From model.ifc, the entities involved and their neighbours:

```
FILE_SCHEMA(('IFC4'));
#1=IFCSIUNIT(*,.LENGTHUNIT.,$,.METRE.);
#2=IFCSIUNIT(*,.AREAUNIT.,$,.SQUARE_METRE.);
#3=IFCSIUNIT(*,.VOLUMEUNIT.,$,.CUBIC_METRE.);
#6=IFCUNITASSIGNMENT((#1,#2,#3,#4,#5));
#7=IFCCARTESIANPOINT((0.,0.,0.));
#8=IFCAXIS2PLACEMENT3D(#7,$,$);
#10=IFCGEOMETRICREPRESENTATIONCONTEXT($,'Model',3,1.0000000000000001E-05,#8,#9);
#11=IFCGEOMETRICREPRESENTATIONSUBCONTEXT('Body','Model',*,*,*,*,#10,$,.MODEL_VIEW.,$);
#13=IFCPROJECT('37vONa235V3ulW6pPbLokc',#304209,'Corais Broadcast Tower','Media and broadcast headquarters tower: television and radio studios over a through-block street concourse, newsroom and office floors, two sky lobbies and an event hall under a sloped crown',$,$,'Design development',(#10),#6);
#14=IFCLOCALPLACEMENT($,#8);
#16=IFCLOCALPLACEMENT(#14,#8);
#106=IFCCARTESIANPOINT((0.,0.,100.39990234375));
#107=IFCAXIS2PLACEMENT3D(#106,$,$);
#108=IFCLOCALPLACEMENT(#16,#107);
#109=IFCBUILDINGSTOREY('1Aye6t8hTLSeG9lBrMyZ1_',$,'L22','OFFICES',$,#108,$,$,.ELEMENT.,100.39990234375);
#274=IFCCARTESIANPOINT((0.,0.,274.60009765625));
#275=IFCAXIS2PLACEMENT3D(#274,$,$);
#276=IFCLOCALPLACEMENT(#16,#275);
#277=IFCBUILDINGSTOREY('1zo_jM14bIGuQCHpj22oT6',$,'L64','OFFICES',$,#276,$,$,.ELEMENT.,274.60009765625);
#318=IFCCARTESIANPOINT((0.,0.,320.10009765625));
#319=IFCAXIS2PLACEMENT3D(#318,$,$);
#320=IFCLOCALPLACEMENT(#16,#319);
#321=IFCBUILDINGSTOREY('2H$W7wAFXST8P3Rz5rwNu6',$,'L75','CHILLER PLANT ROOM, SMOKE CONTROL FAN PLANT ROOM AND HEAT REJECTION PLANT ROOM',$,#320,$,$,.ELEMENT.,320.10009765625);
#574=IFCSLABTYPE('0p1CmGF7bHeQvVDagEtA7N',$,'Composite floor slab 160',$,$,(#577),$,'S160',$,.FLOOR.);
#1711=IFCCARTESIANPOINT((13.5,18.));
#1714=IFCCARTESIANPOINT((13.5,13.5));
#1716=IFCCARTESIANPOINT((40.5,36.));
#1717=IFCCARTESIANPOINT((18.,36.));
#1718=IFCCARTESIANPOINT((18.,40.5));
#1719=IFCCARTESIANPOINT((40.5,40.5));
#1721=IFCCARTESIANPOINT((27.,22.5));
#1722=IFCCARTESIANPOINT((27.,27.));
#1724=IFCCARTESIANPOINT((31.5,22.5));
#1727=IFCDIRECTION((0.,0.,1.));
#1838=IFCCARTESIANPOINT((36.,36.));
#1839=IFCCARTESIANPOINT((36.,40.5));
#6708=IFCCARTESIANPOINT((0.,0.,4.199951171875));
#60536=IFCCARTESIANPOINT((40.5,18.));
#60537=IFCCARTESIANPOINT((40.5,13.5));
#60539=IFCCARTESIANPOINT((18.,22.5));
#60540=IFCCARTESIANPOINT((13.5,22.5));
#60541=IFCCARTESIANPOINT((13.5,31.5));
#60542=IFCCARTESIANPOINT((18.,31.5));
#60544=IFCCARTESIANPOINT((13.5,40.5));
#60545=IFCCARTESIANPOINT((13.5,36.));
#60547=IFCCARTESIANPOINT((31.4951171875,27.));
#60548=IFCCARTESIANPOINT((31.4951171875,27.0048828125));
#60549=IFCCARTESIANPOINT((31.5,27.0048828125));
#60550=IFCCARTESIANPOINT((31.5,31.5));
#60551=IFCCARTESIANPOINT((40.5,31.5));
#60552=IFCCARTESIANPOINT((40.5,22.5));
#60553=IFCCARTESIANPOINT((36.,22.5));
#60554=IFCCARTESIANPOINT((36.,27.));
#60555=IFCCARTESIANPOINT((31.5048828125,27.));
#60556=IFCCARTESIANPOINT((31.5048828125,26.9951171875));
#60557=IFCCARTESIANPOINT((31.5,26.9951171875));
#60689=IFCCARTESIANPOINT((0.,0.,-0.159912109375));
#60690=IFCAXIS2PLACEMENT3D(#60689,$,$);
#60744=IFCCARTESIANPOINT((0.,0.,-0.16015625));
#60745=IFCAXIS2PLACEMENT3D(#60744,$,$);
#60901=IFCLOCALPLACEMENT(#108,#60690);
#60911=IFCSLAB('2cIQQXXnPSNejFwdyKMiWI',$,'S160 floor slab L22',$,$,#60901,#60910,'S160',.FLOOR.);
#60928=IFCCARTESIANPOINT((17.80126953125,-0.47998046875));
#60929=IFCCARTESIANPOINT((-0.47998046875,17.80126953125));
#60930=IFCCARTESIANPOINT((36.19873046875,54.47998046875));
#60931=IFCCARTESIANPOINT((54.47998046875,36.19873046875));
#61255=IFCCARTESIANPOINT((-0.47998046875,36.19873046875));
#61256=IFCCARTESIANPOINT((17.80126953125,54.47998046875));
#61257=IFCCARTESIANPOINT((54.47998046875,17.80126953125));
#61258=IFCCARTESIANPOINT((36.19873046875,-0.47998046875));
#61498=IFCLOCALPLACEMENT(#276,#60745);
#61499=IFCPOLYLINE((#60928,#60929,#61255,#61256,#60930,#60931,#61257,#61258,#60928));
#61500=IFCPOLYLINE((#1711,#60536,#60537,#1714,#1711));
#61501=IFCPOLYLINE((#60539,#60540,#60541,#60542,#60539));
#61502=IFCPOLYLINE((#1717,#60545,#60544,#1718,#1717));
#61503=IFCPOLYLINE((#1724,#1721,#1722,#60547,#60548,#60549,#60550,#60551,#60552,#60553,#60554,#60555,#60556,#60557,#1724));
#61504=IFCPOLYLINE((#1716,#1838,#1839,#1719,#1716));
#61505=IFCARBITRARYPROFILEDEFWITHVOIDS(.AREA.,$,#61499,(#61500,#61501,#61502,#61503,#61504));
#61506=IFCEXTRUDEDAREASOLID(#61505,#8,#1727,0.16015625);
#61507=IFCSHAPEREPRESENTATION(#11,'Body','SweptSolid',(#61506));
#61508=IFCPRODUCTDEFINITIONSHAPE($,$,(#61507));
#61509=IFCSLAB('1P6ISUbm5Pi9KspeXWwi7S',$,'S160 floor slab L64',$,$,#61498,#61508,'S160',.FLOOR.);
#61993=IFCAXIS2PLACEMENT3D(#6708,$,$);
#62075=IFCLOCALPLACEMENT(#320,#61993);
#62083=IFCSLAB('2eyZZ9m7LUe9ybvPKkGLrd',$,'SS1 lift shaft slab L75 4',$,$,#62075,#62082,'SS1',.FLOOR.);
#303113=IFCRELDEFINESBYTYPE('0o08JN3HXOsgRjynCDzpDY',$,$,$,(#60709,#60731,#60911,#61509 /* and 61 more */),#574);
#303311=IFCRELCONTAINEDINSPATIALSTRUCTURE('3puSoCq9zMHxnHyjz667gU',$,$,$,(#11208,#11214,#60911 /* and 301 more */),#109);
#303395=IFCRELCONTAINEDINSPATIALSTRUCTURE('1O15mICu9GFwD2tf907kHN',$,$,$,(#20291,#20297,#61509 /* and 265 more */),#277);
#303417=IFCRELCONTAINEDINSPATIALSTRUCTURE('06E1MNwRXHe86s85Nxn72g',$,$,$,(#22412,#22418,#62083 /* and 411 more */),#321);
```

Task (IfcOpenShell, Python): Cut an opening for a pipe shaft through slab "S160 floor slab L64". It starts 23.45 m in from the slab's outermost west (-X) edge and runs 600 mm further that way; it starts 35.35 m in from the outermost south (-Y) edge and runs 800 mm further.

```python
import numpy as np
import ifcopenshell
import ifcopenshell.api.feature
import ifcopenshell.api.geometry
import ifcopenshell.api.root
import ifcopenshell.geom
import ifcopenshell.util.placement
import ifcopenshell.util.representation
import ifcopenshell.util.shape
import ifcopenshell.util.unit

model = ifcopenshell.open("model.ifc")
unit_scale = ifcopenshell.util.unit.calculate_unit_scale(model)
settings = ifcopenshell.geom.settings()


def volume(element):
    """Net volume in cubic metres, openings subtracted."""
    shape = ifcopenshell.geom.create_shape(settings, element)
    return ifcopenshell.util.shape.get_volume(shape.geometry)


slab = model.by_guid("1P6ISUbm5Pi9KspeXWwi7S")
before = volume(slab)

# Extent in the slab's own axes, in metres. The edges named are its -X and -Y sides.
slab_shape = ifcopenshell.geom.create_shape(settings, slab)
vertices = ifcopenshell.util.shape.get_vertices(slab_shape.geometry)
x_min, y_min, bottom = vertices.min(axis=0)
top = vertices[:, 2].max()

opening = ifcopenshell.api.root.create_entity(model, ifc_class="IfcOpeningElement", name="Pipe shaft opening", predefined_type="OPENING")
context = ifcopenshell.util.representation.get_context(model, "Model", "Body", "MODEL_VIEW")
width, depth = 0.6, 0.8
outline = [(0.0, 0.0), (width, 0.0), (width, depth), (0.0, depth), (0.0, 0.0)]
# Overshoot both faces by 50 mm so the cut is clean.
shape = ifcopenshell.api.geometry.add_slab_representation(
    model, context=context, depth=top - bottom + 0.1, polyline=outline
)
ifcopenshell.api.geometry.assign_representation(model, product=opening, representation=shape)

matrix = ifcopenshell.util.placement.get_local_placement(slab.ObjectPlacement)
matrix[:, 3] = matrix @ np.append(np.array([x_min + 23.45, y_min + 35.35, bottom - 0.05]) / unit_scale, 1.0)
ifcopenshell.api.geometry.edit_object_placement(model, product=opening, matrix=matrix, is_si=False)
ifcopenshell.api.feature.add_feature(model, feature=opening, element=slab)

after = volume(slab)

print(f"slab volume {before:.3f} -> {after:.3f} m3")

model.write("model_edited.ifc")
```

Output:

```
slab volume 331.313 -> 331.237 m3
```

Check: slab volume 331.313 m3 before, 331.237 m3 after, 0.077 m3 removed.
